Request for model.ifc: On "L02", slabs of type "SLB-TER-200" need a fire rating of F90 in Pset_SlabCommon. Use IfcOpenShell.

First a look at what the model holds.

```python
import ifcopenshell
import ifcopenshell.util.element

model = ifcopenshell.open("model.ifc")
print(model.schema)
storey = next(s for s in model.by_type("IfcBuildingStorey") if s.Name == "L02")
slabs = [e for e in ifcopenshell.util.element.get_decomposition(storey) if e.is_a("IfcSlab")]
seen = {}
for e in slabs:
    element_type = ifcopenshell.util.element.get_type(e)
    key = (element_type.Name if element_type != e and element_type else None, ifcopenshell.util.element.get_pset(e, "Pset_SlabCommon", "FireRating"))
    seen[key] = seen.get(key, 0) + 1
for (name, value), count in sorted(seen.items(), key=str):
    print(count, "x", name, "|", value)
```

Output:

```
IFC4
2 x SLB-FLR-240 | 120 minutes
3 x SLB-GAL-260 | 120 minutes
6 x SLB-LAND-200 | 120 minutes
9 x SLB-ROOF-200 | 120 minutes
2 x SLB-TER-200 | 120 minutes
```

```python
import ifcopenshell
import ifcopenshell.api.pset
import ifcopenshell.util.element

model = ifcopenshell.open("model.ifc")

storey = next(s for s in model.by_type("IfcBuildingStorey") if s.Name == "L02")
slabs = [e for e in ifcopenshell.util.element.get_decomposition(storey) if e.is_a("IfcSlab")]

count = 0
for e in slabs:
    element_type = ifcopenshell.util.element.get_type(e)
    if element_type in (None, e) or element_type.Name != "SLB-TER-200":
        continue
    # add_pset returns the element's existing set when there is one.
    pset = ifcopenshell.api.pset.add_pset(model, product=e, name="Pset_SlabCommon")
    ifcopenshell.api.pset.edit_pset(model, pset=pset, properties={"FireRating": "F90"})
    count += 1

print(count, "slabs updated")

model.write("model_edited.ifc")
```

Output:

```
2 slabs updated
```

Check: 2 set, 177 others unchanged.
